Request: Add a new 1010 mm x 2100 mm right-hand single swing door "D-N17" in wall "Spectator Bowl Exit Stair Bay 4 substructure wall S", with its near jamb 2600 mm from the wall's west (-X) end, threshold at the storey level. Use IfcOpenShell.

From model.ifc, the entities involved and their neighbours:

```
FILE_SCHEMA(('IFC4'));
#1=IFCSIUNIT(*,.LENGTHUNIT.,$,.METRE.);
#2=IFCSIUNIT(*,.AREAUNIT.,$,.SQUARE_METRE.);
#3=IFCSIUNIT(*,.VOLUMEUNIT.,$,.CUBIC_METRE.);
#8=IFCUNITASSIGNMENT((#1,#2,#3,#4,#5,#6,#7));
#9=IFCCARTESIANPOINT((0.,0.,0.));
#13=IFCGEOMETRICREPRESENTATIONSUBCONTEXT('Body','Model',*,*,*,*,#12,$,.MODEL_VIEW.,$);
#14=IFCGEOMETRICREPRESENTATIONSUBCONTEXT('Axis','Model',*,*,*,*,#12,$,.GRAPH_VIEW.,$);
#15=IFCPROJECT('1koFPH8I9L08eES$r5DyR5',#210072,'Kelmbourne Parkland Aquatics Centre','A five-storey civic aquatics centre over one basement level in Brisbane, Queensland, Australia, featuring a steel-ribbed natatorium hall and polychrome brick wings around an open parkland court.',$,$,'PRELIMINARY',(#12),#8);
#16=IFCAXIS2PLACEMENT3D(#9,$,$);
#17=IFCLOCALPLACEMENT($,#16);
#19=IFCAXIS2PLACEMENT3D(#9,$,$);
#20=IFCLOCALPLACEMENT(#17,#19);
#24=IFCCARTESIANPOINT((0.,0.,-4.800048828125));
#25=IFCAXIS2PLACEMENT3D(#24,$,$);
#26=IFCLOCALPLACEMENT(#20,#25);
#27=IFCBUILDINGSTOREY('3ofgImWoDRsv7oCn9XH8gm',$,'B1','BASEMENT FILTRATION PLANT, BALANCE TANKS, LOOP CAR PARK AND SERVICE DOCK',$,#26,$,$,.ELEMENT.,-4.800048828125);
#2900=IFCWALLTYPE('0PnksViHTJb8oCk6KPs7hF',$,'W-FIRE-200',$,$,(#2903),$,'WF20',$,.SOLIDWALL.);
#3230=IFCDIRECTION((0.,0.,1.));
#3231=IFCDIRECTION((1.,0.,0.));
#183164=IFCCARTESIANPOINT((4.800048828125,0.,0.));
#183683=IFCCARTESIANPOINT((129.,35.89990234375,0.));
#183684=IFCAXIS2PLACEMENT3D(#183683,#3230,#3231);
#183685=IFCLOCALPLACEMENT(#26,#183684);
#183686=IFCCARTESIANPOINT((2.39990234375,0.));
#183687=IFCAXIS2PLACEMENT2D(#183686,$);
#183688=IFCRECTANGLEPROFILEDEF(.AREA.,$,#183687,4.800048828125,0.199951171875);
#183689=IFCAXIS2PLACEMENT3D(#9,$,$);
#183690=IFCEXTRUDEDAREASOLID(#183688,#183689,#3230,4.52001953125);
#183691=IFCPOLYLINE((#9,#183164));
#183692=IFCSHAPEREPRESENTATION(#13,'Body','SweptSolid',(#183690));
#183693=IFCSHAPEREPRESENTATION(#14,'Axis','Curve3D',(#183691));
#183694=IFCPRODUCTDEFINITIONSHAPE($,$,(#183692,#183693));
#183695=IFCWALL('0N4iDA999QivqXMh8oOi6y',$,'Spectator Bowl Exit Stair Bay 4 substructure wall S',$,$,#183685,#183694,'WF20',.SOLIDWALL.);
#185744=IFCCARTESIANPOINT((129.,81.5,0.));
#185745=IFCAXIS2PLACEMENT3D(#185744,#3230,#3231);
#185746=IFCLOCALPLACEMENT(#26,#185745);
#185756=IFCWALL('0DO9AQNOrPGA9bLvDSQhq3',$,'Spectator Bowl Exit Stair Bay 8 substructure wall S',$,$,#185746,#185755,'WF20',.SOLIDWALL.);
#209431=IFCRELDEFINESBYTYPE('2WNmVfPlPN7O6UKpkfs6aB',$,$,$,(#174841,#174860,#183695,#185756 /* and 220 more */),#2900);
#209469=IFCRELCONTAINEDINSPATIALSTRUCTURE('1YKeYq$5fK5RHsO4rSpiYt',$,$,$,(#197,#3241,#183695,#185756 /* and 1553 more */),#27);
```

```python
import numpy as np
import ifcopenshell
import ifcopenshell.api.feature
import ifcopenshell.api.geometry
import ifcopenshell.api.root
import ifcopenshell.api.spatial
import ifcopenshell.geom
import ifcopenshell.util.element
import ifcopenshell.util.placement
import ifcopenshell.util.representation
import ifcopenshell.util.shape
import ifcopenshell.util.unit

model = ifcopenshell.open("model.ifc")
unit_scale = ifcopenshell.util.unit.calculate_unit_scale(model)
settings = ifcopenshell.geom.settings()


def volume(element):
    """Net volume in cubic metres, openings subtracted."""
    shape = ifcopenshell.geom.create_shape(settings, element)
    return ifcopenshell.util.shape.get_volume(shape.geometry)


wall = model.by_guid("0N4iDA999QivqXMh8oOi6y")
storey = ifcopenshell.util.element.get_container(wall, ifc_class="IfcBuildingStorey")
context = ifcopenshell.util.representation.get_context(model, "Model", "Body", "MODEL_VIEW")
before = volume(wall)

width, height, from_end, sill = 1.01, 2.1, 2.6, 0.0  # metres

# The wall runs along its own X axis, and the end named is its -X end.
wall_shape = ifcopenshell.geom.create_shape(settings, wall)
x, y, z = ifcopenshell.util.shape.get_vertices(wall_shape.geometry).T
start = x.min() + from_end
face, thickness = float(y.min()), float(y.max() - y.min())
wall_matrix = ifcopenshell.util.placement.get_local_placement(wall.ObjectPlacement)
level = ifcopenshell.util.placement.get_local_placement(storey.ObjectPlacement)[2, 3]


def in_wall(x, y):
    """Placement at x, y metres in the wall's axes, at sill height."""
    matrix = wall_matrix.copy()
    matrix[:, 3] = wall_matrix @ np.array([x / unit_scale, y / unit_scale, 0.0, 1.0])
    matrix[2, 3] = level + sill / unit_scale
    return matrix


# Opening: a box that overshoots both wall faces by 50 mm.
opening = ifcopenshell.api.root.create_entity(model, ifc_class="IfcOpeningElement", predefined_type="OPENING")
box = ifcopenshell.api.geometry.add_wall_representation(
    model, context=context, length=width, height=height, thickness=thickness + 0.1
)
ifcopenshell.api.geometry.assign_representation(model, product=opening, representation=box)
ifcopenshell.api.geometry.edit_object_placement(model, product=opening, matrix=in_wall(start, face - 0.05), is_si=False)
ifcopenshell.api.feature.add_feature(model, feature=opening, element=wall)

door = ifcopenshell.api.root.create_entity(model, ifc_class="IfcDoor", name="D-N17", predefined_type="DOOR")
door.OverallWidth, door.OverallHeight = width / unit_scale, height / unit_scale
door.OperationType = "SINGLE_SWING_RIGHT"
body = ifcopenshell.api.geometry.add_door_representation(
    model,
    context=context,
    overall_width=door.OverallWidth,
    overall_height=door.OverallHeight,
    operation_type="SINGLE_SWING_RIGHT",
    lining_properties={"LiningDepth": thickness / unit_scale, "ThresholdDepth": thickness / unit_scale},
)
ifcopenshell.api.geometry.assign_representation(model, product=door, representation=body)
ifcopenshell.api.spatial.assign_container(model, products=[door], relating_structure=storey)
ifcopenshell.api.feature.add_filling(model, opening=opening, element=door)

# The lining spans the wall, so the door starts at the wall face.
ifcopenshell.api.geometry.edit_object_placement(model, product=door, matrix=in_wall(start, face), is_si=False)

after = volume(wall)

print(f"wall volume {before:.3f} -> {after:.3f} m3")

model.write("model_v2.ifc")
```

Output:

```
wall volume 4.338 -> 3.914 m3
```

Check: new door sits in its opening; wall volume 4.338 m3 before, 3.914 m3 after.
